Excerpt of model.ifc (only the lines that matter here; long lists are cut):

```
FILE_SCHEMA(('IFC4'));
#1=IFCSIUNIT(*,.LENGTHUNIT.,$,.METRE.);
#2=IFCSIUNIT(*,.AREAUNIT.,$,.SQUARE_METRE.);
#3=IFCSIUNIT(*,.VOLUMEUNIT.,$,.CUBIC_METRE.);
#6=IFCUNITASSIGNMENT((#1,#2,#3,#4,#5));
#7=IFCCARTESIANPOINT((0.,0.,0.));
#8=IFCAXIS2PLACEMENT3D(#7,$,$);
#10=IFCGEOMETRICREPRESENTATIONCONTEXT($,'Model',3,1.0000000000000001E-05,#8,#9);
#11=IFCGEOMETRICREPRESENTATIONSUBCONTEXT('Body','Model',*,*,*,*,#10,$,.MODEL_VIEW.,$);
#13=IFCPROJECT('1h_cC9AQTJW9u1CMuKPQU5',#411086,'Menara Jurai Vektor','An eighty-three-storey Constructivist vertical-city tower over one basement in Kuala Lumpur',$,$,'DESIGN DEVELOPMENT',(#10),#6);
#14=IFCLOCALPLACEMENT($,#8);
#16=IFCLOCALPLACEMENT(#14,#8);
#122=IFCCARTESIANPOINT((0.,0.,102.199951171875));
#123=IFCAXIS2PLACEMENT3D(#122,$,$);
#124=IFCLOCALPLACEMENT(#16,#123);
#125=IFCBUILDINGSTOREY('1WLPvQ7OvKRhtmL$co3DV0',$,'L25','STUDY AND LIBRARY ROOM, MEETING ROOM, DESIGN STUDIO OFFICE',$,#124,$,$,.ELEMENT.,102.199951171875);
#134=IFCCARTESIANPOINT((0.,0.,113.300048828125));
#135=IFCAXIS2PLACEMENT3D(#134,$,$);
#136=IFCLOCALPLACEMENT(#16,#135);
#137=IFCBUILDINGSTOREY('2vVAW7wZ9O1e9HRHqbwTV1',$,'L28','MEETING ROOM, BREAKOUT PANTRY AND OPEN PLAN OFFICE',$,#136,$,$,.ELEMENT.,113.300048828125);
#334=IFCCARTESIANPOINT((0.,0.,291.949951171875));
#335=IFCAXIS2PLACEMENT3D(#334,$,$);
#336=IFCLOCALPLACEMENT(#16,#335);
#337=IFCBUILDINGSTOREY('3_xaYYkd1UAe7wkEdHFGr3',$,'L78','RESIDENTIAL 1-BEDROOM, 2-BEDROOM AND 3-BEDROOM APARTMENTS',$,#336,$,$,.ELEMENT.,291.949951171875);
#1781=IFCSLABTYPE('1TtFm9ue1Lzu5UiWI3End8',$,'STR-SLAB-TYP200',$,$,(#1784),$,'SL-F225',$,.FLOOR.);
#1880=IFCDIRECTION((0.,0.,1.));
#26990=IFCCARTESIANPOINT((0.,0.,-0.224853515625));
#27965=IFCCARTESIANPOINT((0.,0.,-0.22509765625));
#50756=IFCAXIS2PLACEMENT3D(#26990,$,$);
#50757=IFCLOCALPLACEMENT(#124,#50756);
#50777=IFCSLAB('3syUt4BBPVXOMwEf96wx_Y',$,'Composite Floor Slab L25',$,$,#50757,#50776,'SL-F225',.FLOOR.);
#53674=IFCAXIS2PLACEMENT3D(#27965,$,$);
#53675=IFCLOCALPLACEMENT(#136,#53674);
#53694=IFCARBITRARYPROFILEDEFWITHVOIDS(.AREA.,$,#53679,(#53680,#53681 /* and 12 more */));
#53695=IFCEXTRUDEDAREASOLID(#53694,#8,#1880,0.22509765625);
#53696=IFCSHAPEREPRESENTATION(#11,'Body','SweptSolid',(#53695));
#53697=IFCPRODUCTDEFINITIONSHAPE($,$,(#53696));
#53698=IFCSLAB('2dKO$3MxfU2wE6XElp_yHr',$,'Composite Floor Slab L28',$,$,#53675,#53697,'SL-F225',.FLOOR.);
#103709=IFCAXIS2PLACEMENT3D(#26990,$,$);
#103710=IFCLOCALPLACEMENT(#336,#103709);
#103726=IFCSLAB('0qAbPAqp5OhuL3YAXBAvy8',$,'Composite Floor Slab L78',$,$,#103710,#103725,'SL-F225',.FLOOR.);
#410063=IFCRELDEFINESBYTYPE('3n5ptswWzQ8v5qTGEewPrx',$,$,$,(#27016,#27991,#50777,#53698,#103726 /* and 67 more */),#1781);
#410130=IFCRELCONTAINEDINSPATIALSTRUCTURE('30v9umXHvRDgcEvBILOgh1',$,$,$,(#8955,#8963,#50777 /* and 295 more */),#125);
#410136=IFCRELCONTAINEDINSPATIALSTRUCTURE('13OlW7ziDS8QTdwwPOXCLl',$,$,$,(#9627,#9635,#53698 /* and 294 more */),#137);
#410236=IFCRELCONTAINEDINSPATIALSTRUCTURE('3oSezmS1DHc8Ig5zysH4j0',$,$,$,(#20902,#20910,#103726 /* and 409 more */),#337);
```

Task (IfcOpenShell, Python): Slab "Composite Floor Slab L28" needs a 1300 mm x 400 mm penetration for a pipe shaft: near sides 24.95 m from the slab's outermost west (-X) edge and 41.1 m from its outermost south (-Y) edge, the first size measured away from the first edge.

```python
import numpy as np
import ifcopenshell
import ifcopenshell.api.feature
import ifcopenshell.api.geometry
import ifcopenshell.api.root
import ifcopenshell.geom
import ifcopenshell.util.placement
import ifcopenshell.util.representation
import ifcopenshell.util.shape
import ifcopenshell.util.unit

model = ifcopenshell.open("model.ifc")
unit_scale = ifcopenshell.util.unit.calculate_unit_scale(model)
settings = ifcopenshell.geom.settings()


def volume(element):
    """Net volume in cubic metres, openings subtracted."""
    shape = ifcopenshell.geom.create_shape(settings, element)
    return ifcopenshell.util.shape.get_volume(shape.geometry)


slab = model.by_id(53698)
before = volume(slab)

# Extent in the slab's own axes, in metres. The edges named are its -X and -Y sides.
slab_shape = ifcopenshell.geom.create_shape(settings, slab)
vertices = ifcopenshell.util.shape.get_vertices(slab_shape.geometry)
x_min, y_min, bottom = vertices.min(axis=0)
top = vertices[:, 2].max()

opening = ifcopenshell.api.root.create_entity(model, ifc_class="IfcOpeningElement", name="Pipe shaft opening", predefined_type="OPENING")
context = ifcopenshell.util.representation.get_context(model, "Model", "Body", "MODEL_VIEW")
width, depth = 1.3, 0.4
outline = [(0.0, 0.0), (width, 0.0), (width, depth), (0.0, depth), (0.0, 0.0)]
# Overshoot both faces by 50 mm so the cut is clean.
shape = ifcopenshell.api.geometry.add_slab_representation(
    model, context=context, depth=top - bottom + 0.1, polyline=outline
)
ifcopenshell.api.geometry.assign_representation(model, product=opening, representation=shape)

matrix = ifcopenshell.util.placement.get_local_placement(slab.ObjectPlacement)
matrix[:, 3] = matrix @ np.append(np.array([x_min + 24.95, y_min + 41.1, bottom - 0.05]) / unit_scale, 1.0)
ifcopenshell.api.geometry.edit_object_placement(model, product=opening, matrix=matrix, is_si=False)
ifcopenshell.api.feature.add_feature(model, feature=opening, element=slab)

after = volume(slab)

print(f"slab volume {before:.3f} -> {after:.3f} m3")

model.write("model-out.ifc")
```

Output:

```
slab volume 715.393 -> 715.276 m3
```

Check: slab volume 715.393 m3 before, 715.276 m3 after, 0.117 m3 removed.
